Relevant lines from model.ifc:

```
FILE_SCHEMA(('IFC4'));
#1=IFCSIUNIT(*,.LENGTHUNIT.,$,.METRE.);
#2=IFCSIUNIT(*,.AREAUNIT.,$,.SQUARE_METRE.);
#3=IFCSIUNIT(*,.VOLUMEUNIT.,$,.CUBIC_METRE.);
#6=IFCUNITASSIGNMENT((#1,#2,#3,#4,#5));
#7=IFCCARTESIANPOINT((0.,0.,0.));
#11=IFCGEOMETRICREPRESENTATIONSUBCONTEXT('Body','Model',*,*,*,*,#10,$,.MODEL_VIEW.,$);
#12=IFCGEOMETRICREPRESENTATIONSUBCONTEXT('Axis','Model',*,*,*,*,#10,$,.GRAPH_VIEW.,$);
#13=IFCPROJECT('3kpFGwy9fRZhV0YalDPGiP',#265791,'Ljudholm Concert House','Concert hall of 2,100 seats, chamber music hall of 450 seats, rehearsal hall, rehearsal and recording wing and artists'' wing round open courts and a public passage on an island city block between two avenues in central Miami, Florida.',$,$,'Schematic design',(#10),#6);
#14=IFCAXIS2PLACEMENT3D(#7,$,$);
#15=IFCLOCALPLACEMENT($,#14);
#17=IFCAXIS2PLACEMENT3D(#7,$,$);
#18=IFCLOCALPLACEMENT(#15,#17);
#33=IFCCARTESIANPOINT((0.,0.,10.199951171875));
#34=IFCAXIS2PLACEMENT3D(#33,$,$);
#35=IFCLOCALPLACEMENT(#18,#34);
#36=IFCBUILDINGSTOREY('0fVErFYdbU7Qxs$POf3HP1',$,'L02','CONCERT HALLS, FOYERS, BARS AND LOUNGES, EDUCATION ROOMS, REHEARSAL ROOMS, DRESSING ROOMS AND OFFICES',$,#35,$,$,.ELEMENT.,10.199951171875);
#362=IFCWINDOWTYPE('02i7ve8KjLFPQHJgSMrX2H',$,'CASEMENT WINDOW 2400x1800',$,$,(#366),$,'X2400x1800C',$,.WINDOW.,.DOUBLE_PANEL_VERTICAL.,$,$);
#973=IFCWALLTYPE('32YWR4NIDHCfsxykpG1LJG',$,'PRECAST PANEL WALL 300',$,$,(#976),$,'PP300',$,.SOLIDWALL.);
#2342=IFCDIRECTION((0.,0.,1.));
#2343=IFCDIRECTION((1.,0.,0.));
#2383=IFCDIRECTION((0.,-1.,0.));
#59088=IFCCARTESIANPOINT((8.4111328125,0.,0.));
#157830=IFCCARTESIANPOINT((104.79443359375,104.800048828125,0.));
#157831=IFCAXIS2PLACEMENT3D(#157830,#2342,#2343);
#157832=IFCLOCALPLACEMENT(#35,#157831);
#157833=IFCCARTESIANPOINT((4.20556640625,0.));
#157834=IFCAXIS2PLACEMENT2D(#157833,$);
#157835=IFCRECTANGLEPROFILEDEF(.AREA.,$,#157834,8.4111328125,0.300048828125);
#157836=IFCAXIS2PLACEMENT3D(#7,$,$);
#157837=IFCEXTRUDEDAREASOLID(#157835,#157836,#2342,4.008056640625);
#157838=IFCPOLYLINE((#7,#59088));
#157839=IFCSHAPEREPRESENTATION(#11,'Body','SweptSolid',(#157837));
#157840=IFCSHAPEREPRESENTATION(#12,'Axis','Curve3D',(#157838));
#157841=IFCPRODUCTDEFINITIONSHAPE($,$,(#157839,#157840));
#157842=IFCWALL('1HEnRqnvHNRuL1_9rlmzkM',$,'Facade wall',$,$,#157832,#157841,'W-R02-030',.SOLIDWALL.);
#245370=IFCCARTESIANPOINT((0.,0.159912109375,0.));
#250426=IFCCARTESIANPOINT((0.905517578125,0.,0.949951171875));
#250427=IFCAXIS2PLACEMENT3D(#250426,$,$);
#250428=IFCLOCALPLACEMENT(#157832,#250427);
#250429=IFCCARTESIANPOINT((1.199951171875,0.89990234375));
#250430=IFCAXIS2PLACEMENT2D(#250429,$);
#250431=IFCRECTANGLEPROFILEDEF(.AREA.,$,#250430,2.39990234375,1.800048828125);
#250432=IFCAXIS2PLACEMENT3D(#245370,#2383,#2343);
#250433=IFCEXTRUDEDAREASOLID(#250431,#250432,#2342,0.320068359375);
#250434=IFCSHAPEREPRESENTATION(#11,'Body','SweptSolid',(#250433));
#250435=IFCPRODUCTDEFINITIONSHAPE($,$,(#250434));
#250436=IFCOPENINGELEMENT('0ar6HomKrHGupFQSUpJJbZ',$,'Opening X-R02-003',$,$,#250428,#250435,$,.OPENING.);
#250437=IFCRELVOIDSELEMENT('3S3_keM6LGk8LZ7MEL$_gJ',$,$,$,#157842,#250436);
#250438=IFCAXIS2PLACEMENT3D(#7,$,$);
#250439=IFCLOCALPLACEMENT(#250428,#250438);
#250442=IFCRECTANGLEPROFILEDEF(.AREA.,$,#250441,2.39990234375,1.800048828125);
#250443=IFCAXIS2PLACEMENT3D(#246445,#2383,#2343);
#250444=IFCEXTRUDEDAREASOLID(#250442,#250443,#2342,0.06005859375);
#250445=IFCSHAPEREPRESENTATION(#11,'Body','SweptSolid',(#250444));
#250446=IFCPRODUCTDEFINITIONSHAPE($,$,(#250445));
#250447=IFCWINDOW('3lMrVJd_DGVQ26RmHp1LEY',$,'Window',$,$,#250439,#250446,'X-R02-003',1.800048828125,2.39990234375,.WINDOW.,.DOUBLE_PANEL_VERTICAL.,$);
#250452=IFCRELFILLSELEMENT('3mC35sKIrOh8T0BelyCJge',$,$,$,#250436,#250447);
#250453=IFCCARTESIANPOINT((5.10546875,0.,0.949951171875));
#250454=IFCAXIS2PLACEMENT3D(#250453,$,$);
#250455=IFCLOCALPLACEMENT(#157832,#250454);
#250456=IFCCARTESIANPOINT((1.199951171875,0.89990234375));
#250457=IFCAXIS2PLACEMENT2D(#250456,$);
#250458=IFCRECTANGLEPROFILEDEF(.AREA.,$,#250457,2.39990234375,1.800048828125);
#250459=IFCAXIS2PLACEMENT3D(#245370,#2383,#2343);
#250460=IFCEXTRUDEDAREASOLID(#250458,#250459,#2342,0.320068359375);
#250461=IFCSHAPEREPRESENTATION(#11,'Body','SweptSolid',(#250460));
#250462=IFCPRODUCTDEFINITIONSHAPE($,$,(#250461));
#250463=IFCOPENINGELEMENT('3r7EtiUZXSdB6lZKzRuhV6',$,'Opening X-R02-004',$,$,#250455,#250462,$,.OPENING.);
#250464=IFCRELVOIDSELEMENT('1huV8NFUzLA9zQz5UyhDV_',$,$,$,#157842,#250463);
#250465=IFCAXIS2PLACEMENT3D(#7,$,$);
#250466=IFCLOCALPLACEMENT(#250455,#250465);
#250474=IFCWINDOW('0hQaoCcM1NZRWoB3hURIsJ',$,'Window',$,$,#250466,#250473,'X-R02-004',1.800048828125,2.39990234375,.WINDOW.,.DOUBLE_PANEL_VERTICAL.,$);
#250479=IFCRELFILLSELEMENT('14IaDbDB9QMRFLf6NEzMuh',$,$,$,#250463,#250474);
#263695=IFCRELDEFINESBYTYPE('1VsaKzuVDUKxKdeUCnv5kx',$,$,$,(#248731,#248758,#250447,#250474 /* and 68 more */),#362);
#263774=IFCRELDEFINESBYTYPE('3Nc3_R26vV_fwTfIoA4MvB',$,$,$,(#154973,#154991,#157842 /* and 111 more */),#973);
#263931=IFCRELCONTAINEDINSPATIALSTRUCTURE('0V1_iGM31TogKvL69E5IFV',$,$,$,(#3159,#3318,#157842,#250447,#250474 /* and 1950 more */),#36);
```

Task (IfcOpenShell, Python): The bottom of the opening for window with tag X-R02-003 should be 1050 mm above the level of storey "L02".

```python
import numpy as np
import ifcopenshell
import ifcopenshell.api.geometry
import ifcopenshell.geom
import ifcopenshell.util.element
import ifcopenshell.util.placement
import ifcopenshell.util.shape
import ifcopenshell.util.unit

model = ifcopenshell.open("model.ifc")
unit_scale = ifcopenshell.util.unit.calculate_unit_scale(model)

window = model.by_guid("3lMrVJd_DGVQ26RmHp1LEY")
opening = window.FillsVoids[0].RelatingOpeningElement
storey = ifcopenshell.util.element.get_container(window, ifc_class="IfcBuildingStorey")
level = ifcopenshell.util.placement.get_local_placement(storey.ObjectPlacement)[2, 3]

# The opening's origin need not be at the sill, so measure its lowest point.
shape = ifcopenshell.geom.create_shape(ifcopenshell.geom.settings(), opening)
bottom = ifcopenshell.util.shape.get_shape_bottom_elevation(shape, shape.geometry) / unit_scale
dz = level + 1.05 - bottom

shift = np.array([0.0, 0.0, dz])
# The window is placed relative to its opening, so it follows when the opening moves.
matrix = ifcopenshell.util.placement.get_local_placement(opening.ObjectPlacement)
matrix[:3, 3] += shift
ifcopenshell.api.geometry.edit_object_placement(
    model, product=opening, matrix=matrix, is_si=False, should_transform_children=True
)

print(f"moved by {dz * unit_scale:+.3f} m")

model.write("model_edited.ifc")
```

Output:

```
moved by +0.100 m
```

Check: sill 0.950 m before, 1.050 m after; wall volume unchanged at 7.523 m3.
